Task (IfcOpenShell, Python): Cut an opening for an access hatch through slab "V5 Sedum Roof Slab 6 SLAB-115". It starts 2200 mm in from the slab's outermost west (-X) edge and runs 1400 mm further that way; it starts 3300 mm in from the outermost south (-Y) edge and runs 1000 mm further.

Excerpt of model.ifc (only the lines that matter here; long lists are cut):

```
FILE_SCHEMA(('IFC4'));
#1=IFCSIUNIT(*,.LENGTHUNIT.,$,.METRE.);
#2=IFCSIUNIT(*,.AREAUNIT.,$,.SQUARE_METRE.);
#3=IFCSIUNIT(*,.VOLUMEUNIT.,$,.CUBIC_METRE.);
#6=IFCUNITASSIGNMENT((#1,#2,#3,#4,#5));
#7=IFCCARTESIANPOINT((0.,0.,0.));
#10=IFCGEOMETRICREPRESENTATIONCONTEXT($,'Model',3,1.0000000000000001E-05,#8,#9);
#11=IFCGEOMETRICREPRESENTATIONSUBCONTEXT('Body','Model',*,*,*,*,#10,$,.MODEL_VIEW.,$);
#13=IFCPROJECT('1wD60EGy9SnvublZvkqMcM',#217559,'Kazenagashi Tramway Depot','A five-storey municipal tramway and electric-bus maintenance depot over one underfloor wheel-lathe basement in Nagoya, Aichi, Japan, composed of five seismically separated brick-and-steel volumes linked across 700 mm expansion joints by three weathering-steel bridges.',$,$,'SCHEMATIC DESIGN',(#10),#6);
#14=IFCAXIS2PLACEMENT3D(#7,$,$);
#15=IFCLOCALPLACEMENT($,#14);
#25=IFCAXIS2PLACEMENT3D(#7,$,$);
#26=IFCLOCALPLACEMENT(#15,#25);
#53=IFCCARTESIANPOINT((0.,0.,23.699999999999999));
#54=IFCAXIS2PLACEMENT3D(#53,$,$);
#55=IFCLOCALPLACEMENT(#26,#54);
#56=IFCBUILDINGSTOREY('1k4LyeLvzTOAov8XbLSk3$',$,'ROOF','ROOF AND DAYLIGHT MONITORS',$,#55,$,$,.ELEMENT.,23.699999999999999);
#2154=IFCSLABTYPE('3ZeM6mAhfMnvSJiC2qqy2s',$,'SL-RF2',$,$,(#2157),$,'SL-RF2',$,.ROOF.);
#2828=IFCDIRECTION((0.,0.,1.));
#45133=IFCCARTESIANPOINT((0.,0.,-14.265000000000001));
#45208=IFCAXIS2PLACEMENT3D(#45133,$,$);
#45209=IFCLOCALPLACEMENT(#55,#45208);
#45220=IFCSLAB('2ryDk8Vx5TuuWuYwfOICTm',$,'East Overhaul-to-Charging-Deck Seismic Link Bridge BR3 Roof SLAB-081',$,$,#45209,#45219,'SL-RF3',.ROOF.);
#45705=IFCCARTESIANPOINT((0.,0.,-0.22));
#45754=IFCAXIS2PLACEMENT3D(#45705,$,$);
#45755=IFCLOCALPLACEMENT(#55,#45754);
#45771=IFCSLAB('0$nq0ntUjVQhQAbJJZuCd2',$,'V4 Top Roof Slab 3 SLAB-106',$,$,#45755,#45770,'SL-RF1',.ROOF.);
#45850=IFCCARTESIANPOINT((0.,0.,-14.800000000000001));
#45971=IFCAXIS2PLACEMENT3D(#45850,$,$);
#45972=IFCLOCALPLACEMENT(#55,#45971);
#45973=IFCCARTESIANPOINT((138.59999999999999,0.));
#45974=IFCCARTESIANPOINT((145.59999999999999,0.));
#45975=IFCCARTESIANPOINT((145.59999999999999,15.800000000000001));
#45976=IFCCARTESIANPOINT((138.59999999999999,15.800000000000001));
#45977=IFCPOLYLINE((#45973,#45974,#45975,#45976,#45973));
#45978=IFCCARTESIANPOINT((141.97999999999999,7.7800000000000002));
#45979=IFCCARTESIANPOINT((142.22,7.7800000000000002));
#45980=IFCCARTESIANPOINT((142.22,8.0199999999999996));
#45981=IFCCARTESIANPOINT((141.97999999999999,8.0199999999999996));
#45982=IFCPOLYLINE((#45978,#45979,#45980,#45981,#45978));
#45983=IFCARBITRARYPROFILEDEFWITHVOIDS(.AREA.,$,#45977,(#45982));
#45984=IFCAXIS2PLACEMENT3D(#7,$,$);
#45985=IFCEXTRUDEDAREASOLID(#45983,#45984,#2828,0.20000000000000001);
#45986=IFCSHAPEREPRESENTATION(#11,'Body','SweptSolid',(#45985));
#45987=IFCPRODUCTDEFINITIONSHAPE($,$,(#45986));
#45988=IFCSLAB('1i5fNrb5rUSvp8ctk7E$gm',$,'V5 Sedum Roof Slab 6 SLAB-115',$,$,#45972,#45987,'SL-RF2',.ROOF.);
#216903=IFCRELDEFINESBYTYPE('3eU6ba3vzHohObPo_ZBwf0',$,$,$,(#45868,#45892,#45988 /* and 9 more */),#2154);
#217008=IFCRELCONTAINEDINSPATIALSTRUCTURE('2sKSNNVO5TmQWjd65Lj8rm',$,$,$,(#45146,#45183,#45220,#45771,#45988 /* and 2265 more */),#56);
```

```python
import numpy as np
import ifcopenshell
import ifcopenshell.api.feature
import ifcopenshell.api.geometry
import ifcopenshell.api.root
import ifcopenshell.geom
import ifcopenshell.util.placement
import ifcopenshell.util.representation
import ifcopenshell.util.shape
import ifcopenshell.util.unit

model = ifcopenshell.open("model.ifc")
unit_scale = ifcopenshell.util.unit.calculate_unit_scale(model)
settings = ifcopenshell.geom.settings()


def volume(element):
    """Net volume in cubic metres, openings subtracted."""
    shape = ifcopenshell.geom.create_shape(settings, element)
    return ifcopenshell.util.shape.get_volume(shape.geometry)


slab = model.by_id(45988)
before = volume(slab)

# Extent in the slab's own axes, in metres. The edges named are its -X and -Y sides.
slab_shape = ifcopenshell.geom.create_shape(settings, slab)
vertices = ifcopenshell.util.shape.get_vertices(slab_shape.geometry)
x_min, y_min, bottom = vertices.min(axis=0)
top = vertices[:, 2].max()

opening = ifcopenshell.api.root.create_entity(model, ifc_class="IfcOpeningElement", name="Access hatch opening", predefined_type="OPENING")
context = ifcopenshell.util.representation.get_context(model, "Model", "Body", "MODEL_VIEW")
width, depth = 1.4, 1
outline = [(0.0, 0.0), (width, 0.0), (width, depth), (0.0, depth), (0.0, 0.0)]
# Overshoot both faces by 50 mm so the cut is clean.
shape = ifcopenshell.api.geometry.add_slab_representation(
    model, context=context, depth=top - bottom + 0.1, polyline=outline
)
ifcopenshell.api.geometry.assign_representation(model, product=opening, representation=shape)

matrix = ifcopenshell.util.placement.get_local_placement(slab.ObjectPlacement)
matrix[:, 3] = matrix @ np.append(np.array([x_min + 2.2, y_min + 3.3, bottom - 0.05]) / unit_scale, 1.0)
ifcopenshell.api.geometry.edit_object_placement(model, product=opening, matrix=matrix, is_si=False)
ifcopenshell.api.feature.add_feature(model, feature=opening, element=slab)

after = volume(slab)

print(f"slab volume {before:.3f} -> {after:.3f} m3")

model.write("model_v2.ifc")
```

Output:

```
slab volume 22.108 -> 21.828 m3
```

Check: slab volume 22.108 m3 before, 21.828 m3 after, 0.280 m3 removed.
